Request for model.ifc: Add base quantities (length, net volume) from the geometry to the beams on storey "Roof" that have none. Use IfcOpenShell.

First a look at what the model holds.

```python
import ifcopenshell
import ifcopenshell.util.element
import ifcopenshell.util.unit

model = ifcopenshell.open("model.ifc")
print(model.schema)
for unit_type in ("LENGTHUNIT", "AREAUNIT", "VOLUMEUNIT"):
    print(unit_type, ifcopenshell.util.unit.calculate_unit_scale(model, unit_type))
storey = next(s for s in model.by_type("IfcBuildingStorey") if s.Name == "Roof")
beams = [e for e in ifcopenshell.util.element.get_decomposition(storey) if e.is_a("IfcBeam")]
for e in sorted(beams, key=lambda e: e.id()):
    print(e.id(), e.is_a(), e.Name, list(ifcopenshell.util.element.get_psets(e, qtos_only=True)), sep=" | ")
```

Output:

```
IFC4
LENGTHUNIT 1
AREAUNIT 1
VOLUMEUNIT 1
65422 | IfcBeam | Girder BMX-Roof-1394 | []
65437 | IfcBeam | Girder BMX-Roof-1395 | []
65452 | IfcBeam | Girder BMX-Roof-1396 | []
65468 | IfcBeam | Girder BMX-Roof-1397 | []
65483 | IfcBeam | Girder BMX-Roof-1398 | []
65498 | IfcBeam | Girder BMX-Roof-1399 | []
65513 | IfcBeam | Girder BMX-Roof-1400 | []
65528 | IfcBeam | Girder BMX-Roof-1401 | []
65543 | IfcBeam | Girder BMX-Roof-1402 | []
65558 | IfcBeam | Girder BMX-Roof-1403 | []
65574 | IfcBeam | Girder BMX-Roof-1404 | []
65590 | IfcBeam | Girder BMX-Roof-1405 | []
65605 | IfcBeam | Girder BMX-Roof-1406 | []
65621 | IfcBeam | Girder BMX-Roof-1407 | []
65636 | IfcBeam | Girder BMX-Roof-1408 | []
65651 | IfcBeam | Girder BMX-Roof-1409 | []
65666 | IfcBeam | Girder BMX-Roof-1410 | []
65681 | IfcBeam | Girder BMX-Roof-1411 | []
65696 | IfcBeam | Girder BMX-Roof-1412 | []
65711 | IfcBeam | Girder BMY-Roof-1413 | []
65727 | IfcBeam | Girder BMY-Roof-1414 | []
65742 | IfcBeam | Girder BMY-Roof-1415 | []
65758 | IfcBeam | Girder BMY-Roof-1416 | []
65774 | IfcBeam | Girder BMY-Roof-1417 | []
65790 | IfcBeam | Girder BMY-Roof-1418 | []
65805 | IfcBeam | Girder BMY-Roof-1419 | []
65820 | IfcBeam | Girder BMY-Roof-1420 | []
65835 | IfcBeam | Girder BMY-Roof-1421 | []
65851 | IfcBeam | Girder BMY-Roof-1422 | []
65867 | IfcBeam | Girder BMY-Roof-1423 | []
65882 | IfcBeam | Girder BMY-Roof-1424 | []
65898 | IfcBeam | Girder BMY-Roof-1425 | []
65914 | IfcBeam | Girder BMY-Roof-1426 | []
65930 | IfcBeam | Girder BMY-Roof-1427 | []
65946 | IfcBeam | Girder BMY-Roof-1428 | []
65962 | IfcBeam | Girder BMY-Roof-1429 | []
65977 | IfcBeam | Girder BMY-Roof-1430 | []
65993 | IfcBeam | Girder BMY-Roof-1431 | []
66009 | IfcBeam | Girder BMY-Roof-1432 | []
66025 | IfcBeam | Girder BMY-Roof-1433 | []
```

```python
import ifcopenshell
import ifcopenshell.api.pset
import ifcopenshell.geom
import ifcopenshell.util.element
import ifcopenshell.util.shape
import ifcopenshell.util.unit

model = ifcopenshell.open("model.ifc")
unit_scale = ifcopenshell.util.unit.calculate_unit_scale(model)
volume_scale = ifcopenshell.util.unit.calculate_unit_scale(model, "VOLUMEUNIT")
settings = ifcopenshell.geom.settings()

storey = next(s for s in model.by_type("IfcBuildingStorey") if s.Name == "Roof")
beams = [e for e in ifcopenshell.util.element.get_decomposition(storey) if e.is_a("IfcBeam")]

for e in sorted(beams, key=lambda e: e.id()):
    if ifcopenshell.util.element.get_psets(e, qtos_only=True, should_inherit=False):
        continue
    # Geometry comes back in metres, in the element's own axes.
    shape = ifcopenshell.geom.create_shape(settings, e)
    values = {
        "Length": ifcopenshell.util.shape.get_max_xyz(shape.geometry) / unit_scale,
        "NetVolume": ifcopenshell.util.shape.get_volume(shape.geometry) / volume_scale,
    }
    qto = ifcopenshell.api.pset.add_qto(model, product=e, name="Qto_BeamBaseQuantities")
    ifcopenshell.api.pset.edit_qto(model, qto=qto, properties=values)
    print(e.id(), {k: round(v, 3) for k, v in values.items()})

model.write("model_edited.ifc")
```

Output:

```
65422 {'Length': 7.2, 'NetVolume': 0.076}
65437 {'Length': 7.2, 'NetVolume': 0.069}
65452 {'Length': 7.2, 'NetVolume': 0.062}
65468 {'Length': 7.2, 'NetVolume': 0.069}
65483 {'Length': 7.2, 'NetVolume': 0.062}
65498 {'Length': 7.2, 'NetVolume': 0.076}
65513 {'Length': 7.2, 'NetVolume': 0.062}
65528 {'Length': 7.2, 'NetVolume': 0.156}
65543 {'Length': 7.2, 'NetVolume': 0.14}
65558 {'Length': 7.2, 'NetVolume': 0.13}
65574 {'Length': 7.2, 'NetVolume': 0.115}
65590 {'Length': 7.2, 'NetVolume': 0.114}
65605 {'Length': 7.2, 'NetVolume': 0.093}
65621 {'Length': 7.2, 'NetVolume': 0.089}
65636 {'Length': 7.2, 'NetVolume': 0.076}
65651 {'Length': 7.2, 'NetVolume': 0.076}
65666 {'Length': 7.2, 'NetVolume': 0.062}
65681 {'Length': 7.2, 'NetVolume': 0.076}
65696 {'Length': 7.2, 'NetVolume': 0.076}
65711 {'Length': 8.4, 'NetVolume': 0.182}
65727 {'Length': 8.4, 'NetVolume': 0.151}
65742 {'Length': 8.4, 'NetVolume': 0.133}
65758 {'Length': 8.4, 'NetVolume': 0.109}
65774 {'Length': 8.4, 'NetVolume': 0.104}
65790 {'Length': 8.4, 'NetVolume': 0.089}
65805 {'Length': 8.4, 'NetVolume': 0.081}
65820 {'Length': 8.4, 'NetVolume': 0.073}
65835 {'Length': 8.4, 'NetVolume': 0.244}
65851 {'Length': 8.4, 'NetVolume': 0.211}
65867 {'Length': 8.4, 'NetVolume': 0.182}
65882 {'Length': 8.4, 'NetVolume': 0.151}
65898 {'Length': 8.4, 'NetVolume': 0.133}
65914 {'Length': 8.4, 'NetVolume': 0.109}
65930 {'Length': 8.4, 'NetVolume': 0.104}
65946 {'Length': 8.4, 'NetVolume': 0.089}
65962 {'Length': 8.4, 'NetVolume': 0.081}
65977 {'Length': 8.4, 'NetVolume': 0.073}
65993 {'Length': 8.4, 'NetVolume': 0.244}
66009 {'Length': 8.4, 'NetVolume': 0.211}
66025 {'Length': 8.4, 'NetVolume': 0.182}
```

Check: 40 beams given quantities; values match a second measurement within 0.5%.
